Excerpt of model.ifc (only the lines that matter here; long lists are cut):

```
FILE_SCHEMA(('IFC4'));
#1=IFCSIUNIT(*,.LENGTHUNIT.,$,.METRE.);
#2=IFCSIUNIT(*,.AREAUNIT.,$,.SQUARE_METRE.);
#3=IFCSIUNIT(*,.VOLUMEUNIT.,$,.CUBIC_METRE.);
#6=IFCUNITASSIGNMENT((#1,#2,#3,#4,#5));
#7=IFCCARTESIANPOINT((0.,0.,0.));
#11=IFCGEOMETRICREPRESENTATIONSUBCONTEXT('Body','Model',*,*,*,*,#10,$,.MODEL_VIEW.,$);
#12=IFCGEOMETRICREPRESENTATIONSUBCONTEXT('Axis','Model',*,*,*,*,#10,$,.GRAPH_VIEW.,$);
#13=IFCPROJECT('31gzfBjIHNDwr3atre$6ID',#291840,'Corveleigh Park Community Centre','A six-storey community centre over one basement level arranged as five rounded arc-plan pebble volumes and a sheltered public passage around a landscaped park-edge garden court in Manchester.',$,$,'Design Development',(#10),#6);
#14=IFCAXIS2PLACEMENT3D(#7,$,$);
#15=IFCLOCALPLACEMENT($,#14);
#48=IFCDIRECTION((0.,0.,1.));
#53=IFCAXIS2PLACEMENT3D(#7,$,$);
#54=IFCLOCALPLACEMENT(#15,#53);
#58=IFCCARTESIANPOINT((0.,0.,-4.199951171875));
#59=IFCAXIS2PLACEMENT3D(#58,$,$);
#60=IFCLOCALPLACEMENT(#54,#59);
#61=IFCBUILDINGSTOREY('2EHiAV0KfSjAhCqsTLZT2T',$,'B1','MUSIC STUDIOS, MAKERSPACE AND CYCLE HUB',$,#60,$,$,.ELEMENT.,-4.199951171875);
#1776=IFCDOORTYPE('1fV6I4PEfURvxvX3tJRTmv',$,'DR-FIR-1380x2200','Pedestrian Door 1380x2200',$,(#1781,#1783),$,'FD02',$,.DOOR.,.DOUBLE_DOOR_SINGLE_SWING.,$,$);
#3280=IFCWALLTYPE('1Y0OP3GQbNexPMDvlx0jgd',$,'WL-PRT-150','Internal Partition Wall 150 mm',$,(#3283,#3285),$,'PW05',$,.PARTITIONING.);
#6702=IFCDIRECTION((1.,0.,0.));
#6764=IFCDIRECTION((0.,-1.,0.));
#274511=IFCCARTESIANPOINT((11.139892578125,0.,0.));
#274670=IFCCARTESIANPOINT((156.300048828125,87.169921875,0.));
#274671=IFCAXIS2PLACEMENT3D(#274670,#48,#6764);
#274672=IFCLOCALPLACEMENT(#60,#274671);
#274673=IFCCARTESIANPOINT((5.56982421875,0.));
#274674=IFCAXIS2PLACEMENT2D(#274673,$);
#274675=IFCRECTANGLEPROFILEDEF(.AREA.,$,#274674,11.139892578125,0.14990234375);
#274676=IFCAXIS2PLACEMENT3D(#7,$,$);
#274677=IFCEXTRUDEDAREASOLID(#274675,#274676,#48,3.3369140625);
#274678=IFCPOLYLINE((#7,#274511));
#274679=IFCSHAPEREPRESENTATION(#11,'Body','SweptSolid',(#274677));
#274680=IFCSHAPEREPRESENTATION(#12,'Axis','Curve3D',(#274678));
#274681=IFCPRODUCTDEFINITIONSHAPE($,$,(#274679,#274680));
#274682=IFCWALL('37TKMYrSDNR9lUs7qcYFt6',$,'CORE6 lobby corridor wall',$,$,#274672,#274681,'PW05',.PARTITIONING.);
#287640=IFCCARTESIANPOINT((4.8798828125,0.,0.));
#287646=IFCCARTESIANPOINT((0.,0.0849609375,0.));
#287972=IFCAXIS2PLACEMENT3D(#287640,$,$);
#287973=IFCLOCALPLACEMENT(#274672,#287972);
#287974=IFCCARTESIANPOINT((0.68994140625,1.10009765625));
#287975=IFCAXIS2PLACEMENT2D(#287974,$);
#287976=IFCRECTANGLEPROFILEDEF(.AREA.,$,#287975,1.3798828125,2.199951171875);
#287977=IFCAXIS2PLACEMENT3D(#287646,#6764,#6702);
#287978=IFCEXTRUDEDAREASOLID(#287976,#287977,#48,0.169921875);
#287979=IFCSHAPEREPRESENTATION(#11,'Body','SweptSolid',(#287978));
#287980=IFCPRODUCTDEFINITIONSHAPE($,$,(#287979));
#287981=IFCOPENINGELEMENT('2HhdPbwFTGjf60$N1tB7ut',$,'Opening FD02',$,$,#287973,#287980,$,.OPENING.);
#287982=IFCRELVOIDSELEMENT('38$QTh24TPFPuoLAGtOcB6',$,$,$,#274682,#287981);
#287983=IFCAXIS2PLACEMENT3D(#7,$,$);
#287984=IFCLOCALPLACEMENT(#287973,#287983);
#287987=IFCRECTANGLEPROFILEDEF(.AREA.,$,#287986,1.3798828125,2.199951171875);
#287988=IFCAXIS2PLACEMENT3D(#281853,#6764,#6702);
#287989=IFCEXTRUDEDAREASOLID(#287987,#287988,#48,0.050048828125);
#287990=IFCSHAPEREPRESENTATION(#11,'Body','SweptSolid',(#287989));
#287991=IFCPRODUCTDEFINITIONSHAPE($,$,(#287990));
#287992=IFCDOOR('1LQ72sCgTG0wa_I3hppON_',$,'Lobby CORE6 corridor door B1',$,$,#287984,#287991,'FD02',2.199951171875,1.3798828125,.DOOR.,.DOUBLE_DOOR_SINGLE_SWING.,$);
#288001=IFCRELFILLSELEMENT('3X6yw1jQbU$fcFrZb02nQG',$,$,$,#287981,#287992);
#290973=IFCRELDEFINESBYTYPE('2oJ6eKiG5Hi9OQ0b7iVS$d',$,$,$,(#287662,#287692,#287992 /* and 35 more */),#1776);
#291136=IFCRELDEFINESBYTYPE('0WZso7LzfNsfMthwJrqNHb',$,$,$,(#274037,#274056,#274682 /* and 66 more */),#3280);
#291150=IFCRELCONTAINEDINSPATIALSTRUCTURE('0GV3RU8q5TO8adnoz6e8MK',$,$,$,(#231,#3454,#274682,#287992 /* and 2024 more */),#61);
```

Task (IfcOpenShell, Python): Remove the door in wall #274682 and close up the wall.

```python
import ifcopenshell
import ifcopenshell.api.feature
import ifcopenshell.api.root
import ifcopenshell.geom
import ifcopenshell.util.shape

model = ifcopenshell.open("model.ifc")
settings = ifcopenshell.geom.settings()


def volume(element):
    """Net volume in cubic metres, openings subtracted."""
    shape = ifcopenshell.geom.create_shape(settings, element)
    return ifcopenshell.util.shape.get_volume(shape.geometry)


door = model.by_id(287992)
opening = door.FillsVoids[0].RelatingOpeningElement
wall = opening.VoidsElements[0].RelatingBuildingElement
before = volume(wall)

ifcopenshell.api.root.remove_product(model, product=door)
ifcopenshell.api.feature.remove_feature(model, feature=opening)

after = volume(wall)

print(f"wall volume {before:.3f} -> {after:.3f} m3")

model.write("model-out.ifc")
```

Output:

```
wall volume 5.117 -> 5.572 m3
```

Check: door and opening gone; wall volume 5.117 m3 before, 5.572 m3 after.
